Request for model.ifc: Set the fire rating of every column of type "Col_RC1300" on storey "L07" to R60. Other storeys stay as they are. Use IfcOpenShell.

First a look at what the model holds.

```python
import ifcopenshell
import ifcopenshell.util.element

model = ifcopenshell.open("model.ifc")
print(model.schema)
storey = next(s for s in model.by_type("IfcBuildingStorey") if s.Name == "L07")
columns = [e for e in ifcopenshell.util.element.get_decomposition(storey) if e.is_a("IfcColumn")]
seen = {}
for e in columns:
    element_type = ifcopenshell.util.element.get_type(e)
    key = (element_type.Name if element_type != e and element_type else None, ifcopenshell.util.element.get_pset(e, "Pset_ColumnCommon", "FireRating"))
    seen[key] = seen.get(key, 0) + 1
for (name, value), count in sorted(seen.items(), key=str):
    print(count, "x", name, "|", value)
```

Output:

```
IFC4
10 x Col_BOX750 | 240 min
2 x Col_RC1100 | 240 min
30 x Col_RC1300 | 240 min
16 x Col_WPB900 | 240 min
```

```python
import ifcopenshell
import ifcopenshell.api.pset
import ifcopenshell.util.element

model = ifcopenshell.open("model.ifc")

storey = next(s for s in model.by_type("IfcBuildingStorey") if s.Name == "L07")
columns = [e for e in ifcopenshell.util.element.get_decomposition(storey) if e.is_a("IfcColumn")]

count = 0
for e in columns:
    element_type = ifcopenshell.util.element.get_type(e)
    if element_type in (None, e) or element_type.Name != "Col_RC1300":
        continue
    found = ifcopenshell.util.element.get_pset(e, "Pset_ColumnCommon", should_inherit=False)
    if found:
        pset = model.by_id(found["id"])
        if len(ifcopenshell.util.element.get_elements_by_pset(pset)) > 1:
            pset = ifcopenshell.api.pset.unshare_pset(model, products=[e], pset=pset)[0]
    else:
        pset = ifcopenshell.api.pset.add_pset(model, product=e, name="Pset_ColumnCommon")
    ifcopenshell.api.pset.edit_pset(model, pset=pset, properties={"FireRating": "R60"})
    count += 1

print(count, "columns updated")

model.write("model-out.ifc")
```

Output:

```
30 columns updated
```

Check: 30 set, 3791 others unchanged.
